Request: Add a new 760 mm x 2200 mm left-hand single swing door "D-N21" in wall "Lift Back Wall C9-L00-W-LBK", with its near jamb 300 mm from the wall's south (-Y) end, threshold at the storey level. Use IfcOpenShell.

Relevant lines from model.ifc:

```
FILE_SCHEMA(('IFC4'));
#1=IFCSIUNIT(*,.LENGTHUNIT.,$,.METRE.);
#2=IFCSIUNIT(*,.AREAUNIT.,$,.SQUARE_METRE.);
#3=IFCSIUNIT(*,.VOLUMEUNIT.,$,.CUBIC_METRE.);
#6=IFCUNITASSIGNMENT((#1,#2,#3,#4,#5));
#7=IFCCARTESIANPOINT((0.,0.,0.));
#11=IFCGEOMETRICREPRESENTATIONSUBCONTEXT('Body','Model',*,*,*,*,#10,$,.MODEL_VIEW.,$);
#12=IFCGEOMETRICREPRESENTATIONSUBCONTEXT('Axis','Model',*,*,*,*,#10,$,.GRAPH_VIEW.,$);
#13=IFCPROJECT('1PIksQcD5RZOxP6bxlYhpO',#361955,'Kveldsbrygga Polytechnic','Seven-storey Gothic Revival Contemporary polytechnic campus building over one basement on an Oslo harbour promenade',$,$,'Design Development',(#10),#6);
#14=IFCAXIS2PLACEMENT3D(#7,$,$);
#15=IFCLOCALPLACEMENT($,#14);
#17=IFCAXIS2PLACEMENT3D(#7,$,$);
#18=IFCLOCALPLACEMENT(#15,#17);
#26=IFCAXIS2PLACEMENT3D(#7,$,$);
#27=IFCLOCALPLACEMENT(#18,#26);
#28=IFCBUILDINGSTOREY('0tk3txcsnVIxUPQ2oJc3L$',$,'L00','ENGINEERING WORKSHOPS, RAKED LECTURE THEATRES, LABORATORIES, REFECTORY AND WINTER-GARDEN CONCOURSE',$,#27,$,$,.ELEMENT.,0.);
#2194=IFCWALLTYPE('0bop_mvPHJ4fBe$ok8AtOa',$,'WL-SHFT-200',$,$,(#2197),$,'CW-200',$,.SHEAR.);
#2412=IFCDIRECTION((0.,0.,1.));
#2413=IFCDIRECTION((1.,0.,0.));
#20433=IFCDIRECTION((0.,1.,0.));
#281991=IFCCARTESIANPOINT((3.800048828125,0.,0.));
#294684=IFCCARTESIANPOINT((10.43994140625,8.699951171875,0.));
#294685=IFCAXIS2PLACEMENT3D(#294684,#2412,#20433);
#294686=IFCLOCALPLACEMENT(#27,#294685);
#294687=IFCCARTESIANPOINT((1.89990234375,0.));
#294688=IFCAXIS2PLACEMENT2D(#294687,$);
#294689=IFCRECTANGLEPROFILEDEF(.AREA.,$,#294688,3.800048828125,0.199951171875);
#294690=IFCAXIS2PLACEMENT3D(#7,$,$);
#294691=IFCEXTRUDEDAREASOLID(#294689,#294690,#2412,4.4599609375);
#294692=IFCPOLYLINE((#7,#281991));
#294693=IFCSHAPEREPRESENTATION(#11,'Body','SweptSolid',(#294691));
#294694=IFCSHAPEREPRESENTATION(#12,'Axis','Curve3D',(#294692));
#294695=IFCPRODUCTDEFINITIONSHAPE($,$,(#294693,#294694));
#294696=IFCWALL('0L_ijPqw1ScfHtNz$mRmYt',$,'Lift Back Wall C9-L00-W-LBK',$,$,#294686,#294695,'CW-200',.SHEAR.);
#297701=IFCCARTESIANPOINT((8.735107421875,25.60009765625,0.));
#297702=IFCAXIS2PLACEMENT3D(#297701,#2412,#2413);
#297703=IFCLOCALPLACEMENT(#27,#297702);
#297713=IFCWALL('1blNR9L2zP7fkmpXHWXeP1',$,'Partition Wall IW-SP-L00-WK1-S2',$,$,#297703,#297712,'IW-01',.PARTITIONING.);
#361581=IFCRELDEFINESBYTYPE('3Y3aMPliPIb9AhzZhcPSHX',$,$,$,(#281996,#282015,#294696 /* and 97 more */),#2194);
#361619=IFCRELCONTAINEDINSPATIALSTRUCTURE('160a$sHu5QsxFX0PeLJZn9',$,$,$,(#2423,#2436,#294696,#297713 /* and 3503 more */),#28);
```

```python
import numpy as np
import ifcopenshell
import ifcopenshell.api.feature
import ifcopenshell.api.geometry
import ifcopenshell.api.root
import ifcopenshell.api.spatial
import ifcopenshell.geom
import ifcopenshell.util.element
import ifcopenshell.util.placement
import ifcopenshell.util.representation
import ifcopenshell.util.shape
import ifcopenshell.util.unit

model = ifcopenshell.open("model.ifc")
unit_scale = ifcopenshell.util.unit.calculate_unit_scale(model)
settings = ifcopenshell.geom.settings()


def volume(element):
    """Net volume in cubic metres, openings subtracted."""
    shape = ifcopenshell.geom.create_shape(settings, element)
    return ifcopenshell.util.shape.get_volume(shape.geometry)


wall = model.by_guid("0L_ijPqw1ScfHtNz$mRmYt")
storey = ifcopenshell.util.element.get_container(wall, ifc_class="IfcBuildingStorey")
context = ifcopenshell.util.representation.get_context(model, "Model", "Body", "MODEL_VIEW")
before = volume(wall)

width, height, from_end, sill = 0.76, 2.2, 0.3, 0.0  # metres

# The wall runs along its own X axis, and the end named is its -X end.
wall_shape = ifcopenshell.geom.create_shape(settings, wall)
x, y, z = ifcopenshell.util.shape.get_vertices(wall_shape.geometry).T
start = x.min() + from_end
face, thickness = float(y.min()), float(y.max() - y.min())
wall_matrix = ifcopenshell.util.placement.get_local_placement(wall.ObjectPlacement)
level = ifcopenshell.util.placement.get_local_placement(storey.ObjectPlacement)[2, 3]


def in_wall(x, y):
    """Placement at x, y metres in the wall's axes, at sill height."""
    matrix = wall_matrix.copy()
    matrix[:, 3] = wall_matrix @ np.array([x / unit_scale, y / unit_scale, 0.0, 1.0])
    matrix[2, 3] = level + sill / unit_scale
    return matrix


# Opening: a box that overshoots both wall faces by 50 mm.
opening = ifcopenshell.api.root.create_entity(model, ifc_class="IfcOpeningElement", predefined_type="OPENING")
box = ifcopenshell.api.geometry.add_wall_representation(
    model, context=context, length=width, height=height, thickness=thickness + 0.1
)
ifcopenshell.api.geometry.assign_representation(model, product=opening, representation=box)
ifcopenshell.api.geometry.edit_object_placement(model, product=opening, matrix=in_wall(start, face - 0.05), is_si=False)
ifcopenshell.api.feature.add_feature(model, feature=opening, element=wall)

door = ifcopenshell.api.root.create_entity(model, ifc_class="IfcDoor", name="D-N21", predefined_type="DOOR")
door.OverallWidth, door.OverallHeight = width / unit_scale, height / unit_scale
door.OperationType = "SINGLE_SWING_LEFT"
body = ifcopenshell.api.geometry.add_door_representation(
    model,
    context=context,
    overall_width=door.OverallWidth,
    overall_height=door.OverallHeight,
    operation_type="SINGLE_SWING_LEFT",
    lining_properties={"LiningDepth": thickness / unit_scale, "ThresholdDepth": thickness / unit_scale},
)
ifcopenshell.api.geometry.assign_representation(model, product=door, representation=body)
ifcopenshell.api.spatial.assign_container(model, products=[door], relating_structure=storey)
ifcopenshell.api.feature.add_filling(model, opening=opening, element=door)

# The lining spans the wall, so the door starts at the wall face.
ifcopenshell.api.geometry.edit_object_placement(model, product=door, matrix=in_wall(start, face), is_si=False)

after = volume(wall)

print(f"wall volume {before:.3f} -> {after:.3f} m3")

model.write("model_edited.ifc")
```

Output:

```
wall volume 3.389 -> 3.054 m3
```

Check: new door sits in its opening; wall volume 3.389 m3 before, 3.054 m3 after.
